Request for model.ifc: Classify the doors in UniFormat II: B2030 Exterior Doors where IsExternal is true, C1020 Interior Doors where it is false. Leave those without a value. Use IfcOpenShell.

First a look at what the model holds.

```python
import ifcopenshell
import ifcopenshell.util.element

model = ifcopenshell.open("model.ifc")
print(model.schema)
print("classifications:", [c.Name for c in model.by_type("IfcClassification")])
values = [ifcopenshell.util.element.get_pset(e, "Pset_DoorCommon", "IsExternal") for e in model.by_type("IfcDoor")]
for value in (True, False, None):
    print("IsExternal", value, values.count(value))
```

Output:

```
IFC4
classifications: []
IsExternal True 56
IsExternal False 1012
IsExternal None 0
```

```python
import ifcopenshell
import ifcopenshell.api.classification
import ifcopenshell.util.element

model = ifcopenshell.open("model.ifc")

system = ifcopenshell.api.classification.add_classification(model, classification="UniFormat II")

doors = model.by_type("IfcDoor")
external = {e: ifcopenshell.util.element.get_pset(e, "Pset_DoorCommon", "IsExternal") for e in doors}
for flag, code, name in ((True, "B2030", "Exterior Doors"), (False, "C1020", "Interior Doors")):
    products = [e for e in doors if external[e] is flag]
    ifcopenshell.api.classification.add_reference(
        model, products=products, classification=system, identification=code, name=name
    )
    print(code, len(products))

model.write("model_edited.ifc")
```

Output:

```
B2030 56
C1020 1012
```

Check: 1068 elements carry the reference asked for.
